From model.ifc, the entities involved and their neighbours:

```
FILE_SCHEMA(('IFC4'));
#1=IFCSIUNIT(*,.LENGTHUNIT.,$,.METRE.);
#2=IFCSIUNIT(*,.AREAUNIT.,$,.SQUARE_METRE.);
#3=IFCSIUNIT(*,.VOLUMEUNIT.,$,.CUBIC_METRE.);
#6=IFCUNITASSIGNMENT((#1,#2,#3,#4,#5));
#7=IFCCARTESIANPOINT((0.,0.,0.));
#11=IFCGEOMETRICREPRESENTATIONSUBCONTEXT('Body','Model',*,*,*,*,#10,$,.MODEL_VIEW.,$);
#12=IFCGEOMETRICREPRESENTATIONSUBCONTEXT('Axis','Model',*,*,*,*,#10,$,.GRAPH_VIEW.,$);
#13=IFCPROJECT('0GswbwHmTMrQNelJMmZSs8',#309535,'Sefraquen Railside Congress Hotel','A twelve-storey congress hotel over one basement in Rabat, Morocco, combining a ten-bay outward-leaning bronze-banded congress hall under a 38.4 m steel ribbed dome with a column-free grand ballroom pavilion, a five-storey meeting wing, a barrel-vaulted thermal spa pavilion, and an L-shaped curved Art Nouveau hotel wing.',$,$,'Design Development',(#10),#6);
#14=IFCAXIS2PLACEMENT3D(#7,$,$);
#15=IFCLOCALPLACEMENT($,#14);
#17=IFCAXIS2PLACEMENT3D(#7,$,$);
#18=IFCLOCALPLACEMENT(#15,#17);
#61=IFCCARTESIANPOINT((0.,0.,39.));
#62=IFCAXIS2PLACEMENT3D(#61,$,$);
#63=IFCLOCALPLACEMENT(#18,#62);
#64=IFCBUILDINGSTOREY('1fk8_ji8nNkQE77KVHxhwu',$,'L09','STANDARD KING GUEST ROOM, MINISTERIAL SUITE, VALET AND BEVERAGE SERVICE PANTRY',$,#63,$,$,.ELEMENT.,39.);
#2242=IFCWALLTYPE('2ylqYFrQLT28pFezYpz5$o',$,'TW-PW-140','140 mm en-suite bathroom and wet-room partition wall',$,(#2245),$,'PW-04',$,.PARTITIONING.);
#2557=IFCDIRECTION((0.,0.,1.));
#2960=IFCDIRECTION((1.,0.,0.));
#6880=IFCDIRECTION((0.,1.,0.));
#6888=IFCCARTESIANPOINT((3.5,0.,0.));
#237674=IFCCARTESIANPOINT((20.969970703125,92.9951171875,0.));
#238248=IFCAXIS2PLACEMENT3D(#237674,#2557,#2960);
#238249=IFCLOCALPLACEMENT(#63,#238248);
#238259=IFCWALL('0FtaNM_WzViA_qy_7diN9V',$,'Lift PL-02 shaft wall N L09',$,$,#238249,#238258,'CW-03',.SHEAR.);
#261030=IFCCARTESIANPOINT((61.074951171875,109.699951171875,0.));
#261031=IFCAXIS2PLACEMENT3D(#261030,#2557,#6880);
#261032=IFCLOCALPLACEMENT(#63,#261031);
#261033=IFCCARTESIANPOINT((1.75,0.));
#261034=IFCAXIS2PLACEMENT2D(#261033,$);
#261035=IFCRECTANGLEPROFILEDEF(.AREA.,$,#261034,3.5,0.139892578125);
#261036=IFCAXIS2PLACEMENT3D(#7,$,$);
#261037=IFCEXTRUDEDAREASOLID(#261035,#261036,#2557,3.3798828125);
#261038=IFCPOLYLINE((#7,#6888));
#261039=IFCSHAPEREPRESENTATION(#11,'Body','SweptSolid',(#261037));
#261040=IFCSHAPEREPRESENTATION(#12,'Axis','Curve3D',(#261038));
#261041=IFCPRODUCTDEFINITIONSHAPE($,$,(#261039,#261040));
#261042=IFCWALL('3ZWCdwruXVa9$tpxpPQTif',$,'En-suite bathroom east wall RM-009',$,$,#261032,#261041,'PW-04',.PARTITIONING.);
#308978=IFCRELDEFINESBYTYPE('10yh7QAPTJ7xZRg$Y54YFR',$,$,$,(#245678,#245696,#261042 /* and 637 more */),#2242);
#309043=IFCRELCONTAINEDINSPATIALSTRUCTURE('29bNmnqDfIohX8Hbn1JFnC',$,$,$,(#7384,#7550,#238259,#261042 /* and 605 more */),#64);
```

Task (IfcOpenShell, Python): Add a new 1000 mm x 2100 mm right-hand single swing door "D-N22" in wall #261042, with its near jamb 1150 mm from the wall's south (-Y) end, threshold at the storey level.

```python
import numpy as np
import ifcopenshell
import ifcopenshell.api.feature
import ifcopenshell.api.geometry
import ifcopenshell.api.root
import ifcopenshell.api.spatial
import ifcopenshell.geom
import ifcopenshell.util.element
import ifcopenshell.util.placement
import ifcopenshell.util.representation
import ifcopenshell.util.shape
import ifcopenshell.util.unit

model = ifcopenshell.open("model.ifc")
unit_scale = ifcopenshell.util.unit.calculate_unit_scale(model)
settings = ifcopenshell.geom.settings()


def volume(element):
    """Net volume in cubic metres, openings subtracted."""
    shape = ifcopenshell.geom.create_shape(settings, element)
    return ifcopenshell.util.shape.get_volume(shape.geometry)


wall = model.by_guid("3ZWCdwruXVa9$tpxpPQTif")
storey = ifcopenshell.util.element.get_container(wall, ifc_class="IfcBuildingStorey")
context = ifcopenshell.util.representation.get_context(model, "Model", "Body", "MODEL_VIEW")
before = volume(wall)

width, height, from_end, sill = 1, 2.1, 1.15, 0.0  # metres

# The wall runs along its own X axis, and the end named is its -X end.
wall_shape = ifcopenshell.geom.create_shape(settings, wall)
x, y, z = ifcopenshell.util.shape.get_vertices(wall_shape.geometry).T
start = x.min() + from_end
face, thickness = float(y.min()), float(y.max() - y.min())
wall_matrix = ifcopenshell.util.placement.get_local_placement(wall.ObjectPlacement)
level = ifcopenshell.util.placement.get_local_placement(storey.ObjectPlacement)[2, 3]


def in_wall(x, y):
    """Placement at x, y metres in the wall's axes, at sill height."""
    matrix = wall_matrix.copy()
    matrix[:, 3] = wall_matrix @ np.array([x / unit_scale, y / unit_scale, 0.0, 1.0])
    matrix[2, 3] = level + sill / unit_scale
    return matrix


# Opening: a box that overshoots both wall faces by 50 mm.
opening = ifcopenshell.api.root.create_entity(model, ifc_class="IfcOpeningElement", predefined_type="OPENING")
box = ifcopenshell.api.geometry.add_wall_representation(
    model, context=context, length=width, height=height, thickness=thickness + 0.1
)
ifcopenshell.api.geometry.assign_representation(model, product=opening, representation=box)
ifcopenshell.api.geometry.edit_object_placement(model, product=opening, matrix=in_wall(start, face - 0.05), is_si=False)
ifcopenshell.api.feature.add_feature(model, feature=opening, element=wall)

door = ifcopenshell.api.root.create_entity(model, ifc_class="IfcDoor", name="D-N22", predefined_type="DOOR")
door.OverallWidth, door.OverallHeight = width / unit_scale, height / unit_scale
door.OperationType = "SINGLE_SWING_RIGHT"
body = ifcopenshell.api.geometry.add_door_representation(
    model,
    context=context,
    overall_width=door.OverallWidth,
    overall_height=door.OverallHeight,
    operation_type="SINGLE_SWING_RIGHT",
    lining_properties={"LiningDepth": thickness / unit_scale, "ThresholdDepth": thickness / unit_scale},
)
ifcopenshell.api.geometry.assign_representation(model, product=door, representation=body)
ifcopenshell.api.spatial.assign_container(model, products=[door], relating_structure=storey)
ifcopenshell.api.feature.add_filling(model, opening=opening, element=door)

# The lining spans the wall, so the door starts at the wall face.
ifcopenshell.api.geometry.edit_object_placement(model, product=door, matrix=in_wall(start, face), is_si=False)

after = volume(wall)

print(f"wall volume {before:.3f} -> {after:.3f} m3")

model.write("model_updated.ifc")
```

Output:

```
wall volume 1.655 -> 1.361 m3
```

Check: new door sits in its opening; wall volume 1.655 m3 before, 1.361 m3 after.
